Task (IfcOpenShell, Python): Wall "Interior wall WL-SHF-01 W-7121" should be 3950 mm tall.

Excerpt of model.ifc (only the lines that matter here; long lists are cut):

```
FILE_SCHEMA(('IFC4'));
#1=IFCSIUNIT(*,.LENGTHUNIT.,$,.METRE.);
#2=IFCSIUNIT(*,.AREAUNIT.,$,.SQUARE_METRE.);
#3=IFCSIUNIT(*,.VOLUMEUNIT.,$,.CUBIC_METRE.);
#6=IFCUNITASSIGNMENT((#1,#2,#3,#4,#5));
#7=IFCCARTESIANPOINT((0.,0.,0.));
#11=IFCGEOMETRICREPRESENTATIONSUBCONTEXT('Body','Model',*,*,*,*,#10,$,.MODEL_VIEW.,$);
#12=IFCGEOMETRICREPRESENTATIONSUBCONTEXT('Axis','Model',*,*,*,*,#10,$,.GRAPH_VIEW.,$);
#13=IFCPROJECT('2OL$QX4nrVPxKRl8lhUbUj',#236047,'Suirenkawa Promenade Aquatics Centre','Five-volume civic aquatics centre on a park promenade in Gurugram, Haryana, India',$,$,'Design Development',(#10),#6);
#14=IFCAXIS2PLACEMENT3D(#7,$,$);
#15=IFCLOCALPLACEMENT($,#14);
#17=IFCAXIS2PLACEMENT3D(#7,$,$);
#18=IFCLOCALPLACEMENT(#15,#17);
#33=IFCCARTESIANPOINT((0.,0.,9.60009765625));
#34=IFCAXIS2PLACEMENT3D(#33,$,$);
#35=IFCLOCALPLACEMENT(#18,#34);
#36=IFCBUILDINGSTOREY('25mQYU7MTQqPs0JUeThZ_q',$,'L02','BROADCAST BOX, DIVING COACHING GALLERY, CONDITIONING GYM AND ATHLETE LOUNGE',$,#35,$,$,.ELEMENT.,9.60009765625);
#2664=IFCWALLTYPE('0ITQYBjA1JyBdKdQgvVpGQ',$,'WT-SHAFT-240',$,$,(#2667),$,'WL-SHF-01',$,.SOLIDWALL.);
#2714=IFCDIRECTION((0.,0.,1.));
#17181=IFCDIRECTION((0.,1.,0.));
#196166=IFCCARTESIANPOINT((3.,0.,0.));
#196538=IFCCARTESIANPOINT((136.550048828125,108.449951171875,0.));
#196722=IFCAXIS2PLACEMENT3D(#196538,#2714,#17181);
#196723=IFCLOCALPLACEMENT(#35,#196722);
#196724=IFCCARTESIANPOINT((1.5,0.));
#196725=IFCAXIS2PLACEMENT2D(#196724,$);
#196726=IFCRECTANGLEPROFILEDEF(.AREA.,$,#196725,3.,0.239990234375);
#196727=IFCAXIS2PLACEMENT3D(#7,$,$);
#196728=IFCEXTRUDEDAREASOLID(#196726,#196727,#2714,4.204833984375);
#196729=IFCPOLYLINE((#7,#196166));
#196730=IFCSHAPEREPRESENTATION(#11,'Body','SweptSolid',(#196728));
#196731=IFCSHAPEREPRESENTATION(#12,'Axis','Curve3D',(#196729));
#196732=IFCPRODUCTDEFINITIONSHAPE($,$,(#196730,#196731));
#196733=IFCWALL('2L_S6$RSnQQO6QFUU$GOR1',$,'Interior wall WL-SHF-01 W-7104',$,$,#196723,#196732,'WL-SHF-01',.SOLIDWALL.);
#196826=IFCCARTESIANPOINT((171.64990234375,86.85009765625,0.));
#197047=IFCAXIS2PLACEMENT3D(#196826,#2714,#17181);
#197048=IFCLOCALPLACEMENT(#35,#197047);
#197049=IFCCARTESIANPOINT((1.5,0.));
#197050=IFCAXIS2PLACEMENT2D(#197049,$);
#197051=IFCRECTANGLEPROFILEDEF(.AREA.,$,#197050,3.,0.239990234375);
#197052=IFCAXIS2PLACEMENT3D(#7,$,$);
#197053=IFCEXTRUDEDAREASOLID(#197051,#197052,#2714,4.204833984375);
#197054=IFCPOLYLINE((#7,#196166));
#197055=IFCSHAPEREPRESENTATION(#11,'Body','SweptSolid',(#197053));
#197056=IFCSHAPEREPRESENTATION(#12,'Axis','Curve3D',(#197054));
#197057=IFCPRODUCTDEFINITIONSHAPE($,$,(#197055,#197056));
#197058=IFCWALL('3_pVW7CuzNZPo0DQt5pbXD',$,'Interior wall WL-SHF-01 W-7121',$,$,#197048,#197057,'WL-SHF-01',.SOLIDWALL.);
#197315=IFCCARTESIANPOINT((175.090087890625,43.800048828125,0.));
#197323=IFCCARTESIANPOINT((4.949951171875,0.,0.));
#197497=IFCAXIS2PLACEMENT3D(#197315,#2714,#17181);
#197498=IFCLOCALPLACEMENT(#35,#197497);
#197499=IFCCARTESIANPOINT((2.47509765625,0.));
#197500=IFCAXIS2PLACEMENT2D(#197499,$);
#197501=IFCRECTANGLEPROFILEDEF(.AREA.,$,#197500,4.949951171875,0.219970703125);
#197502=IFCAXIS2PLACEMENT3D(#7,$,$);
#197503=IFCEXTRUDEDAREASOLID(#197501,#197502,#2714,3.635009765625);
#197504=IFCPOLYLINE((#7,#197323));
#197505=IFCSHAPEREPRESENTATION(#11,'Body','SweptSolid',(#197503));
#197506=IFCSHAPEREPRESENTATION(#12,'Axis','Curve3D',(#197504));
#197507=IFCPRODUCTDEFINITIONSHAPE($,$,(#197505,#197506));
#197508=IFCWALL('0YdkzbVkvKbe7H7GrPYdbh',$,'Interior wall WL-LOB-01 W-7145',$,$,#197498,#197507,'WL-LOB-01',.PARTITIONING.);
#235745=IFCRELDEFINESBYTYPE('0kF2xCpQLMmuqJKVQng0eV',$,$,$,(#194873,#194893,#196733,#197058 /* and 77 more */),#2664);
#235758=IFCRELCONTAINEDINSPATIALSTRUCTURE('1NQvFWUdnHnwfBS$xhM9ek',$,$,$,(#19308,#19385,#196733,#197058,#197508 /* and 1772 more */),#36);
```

```python
import ifcopenshell
import ifcopenshell.geom
import ifcopenshell.util.representation
import ifcopenshell.util.shape
import ifcopenshell.util.unit

model = ifcopenshell.open("model.ifc")
unit_scale = ifcopenshell.util.unit.calculate_unit_scale(model)
settings = ifcopenshell.geom.settings()


def volume(element):
    """Net volume in cubic metres, openings subtracted."""
    shape = ifcopenshell.geom.create_shape(settings, element)
    return ifcopenshell.util.shape.get_volume(shape.geometry)


wall = model.by_id(197058)
before = volume(wall)

body = ifcopenshell.util.representation.get_representation(wall, "Model", "Body")
solid = body.Items[0]
old_height = solid.Depth
solid.Depth = 3.95 / unit_scale
after = volume(wall)

print(f"height {old_height:g} -> {solid.Depth:g}, volume {before:.3f} -> {after:.3f} m3")

model.write("model_v2.ifc")
```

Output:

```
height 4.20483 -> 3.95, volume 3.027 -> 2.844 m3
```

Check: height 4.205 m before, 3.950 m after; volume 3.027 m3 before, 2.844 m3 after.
